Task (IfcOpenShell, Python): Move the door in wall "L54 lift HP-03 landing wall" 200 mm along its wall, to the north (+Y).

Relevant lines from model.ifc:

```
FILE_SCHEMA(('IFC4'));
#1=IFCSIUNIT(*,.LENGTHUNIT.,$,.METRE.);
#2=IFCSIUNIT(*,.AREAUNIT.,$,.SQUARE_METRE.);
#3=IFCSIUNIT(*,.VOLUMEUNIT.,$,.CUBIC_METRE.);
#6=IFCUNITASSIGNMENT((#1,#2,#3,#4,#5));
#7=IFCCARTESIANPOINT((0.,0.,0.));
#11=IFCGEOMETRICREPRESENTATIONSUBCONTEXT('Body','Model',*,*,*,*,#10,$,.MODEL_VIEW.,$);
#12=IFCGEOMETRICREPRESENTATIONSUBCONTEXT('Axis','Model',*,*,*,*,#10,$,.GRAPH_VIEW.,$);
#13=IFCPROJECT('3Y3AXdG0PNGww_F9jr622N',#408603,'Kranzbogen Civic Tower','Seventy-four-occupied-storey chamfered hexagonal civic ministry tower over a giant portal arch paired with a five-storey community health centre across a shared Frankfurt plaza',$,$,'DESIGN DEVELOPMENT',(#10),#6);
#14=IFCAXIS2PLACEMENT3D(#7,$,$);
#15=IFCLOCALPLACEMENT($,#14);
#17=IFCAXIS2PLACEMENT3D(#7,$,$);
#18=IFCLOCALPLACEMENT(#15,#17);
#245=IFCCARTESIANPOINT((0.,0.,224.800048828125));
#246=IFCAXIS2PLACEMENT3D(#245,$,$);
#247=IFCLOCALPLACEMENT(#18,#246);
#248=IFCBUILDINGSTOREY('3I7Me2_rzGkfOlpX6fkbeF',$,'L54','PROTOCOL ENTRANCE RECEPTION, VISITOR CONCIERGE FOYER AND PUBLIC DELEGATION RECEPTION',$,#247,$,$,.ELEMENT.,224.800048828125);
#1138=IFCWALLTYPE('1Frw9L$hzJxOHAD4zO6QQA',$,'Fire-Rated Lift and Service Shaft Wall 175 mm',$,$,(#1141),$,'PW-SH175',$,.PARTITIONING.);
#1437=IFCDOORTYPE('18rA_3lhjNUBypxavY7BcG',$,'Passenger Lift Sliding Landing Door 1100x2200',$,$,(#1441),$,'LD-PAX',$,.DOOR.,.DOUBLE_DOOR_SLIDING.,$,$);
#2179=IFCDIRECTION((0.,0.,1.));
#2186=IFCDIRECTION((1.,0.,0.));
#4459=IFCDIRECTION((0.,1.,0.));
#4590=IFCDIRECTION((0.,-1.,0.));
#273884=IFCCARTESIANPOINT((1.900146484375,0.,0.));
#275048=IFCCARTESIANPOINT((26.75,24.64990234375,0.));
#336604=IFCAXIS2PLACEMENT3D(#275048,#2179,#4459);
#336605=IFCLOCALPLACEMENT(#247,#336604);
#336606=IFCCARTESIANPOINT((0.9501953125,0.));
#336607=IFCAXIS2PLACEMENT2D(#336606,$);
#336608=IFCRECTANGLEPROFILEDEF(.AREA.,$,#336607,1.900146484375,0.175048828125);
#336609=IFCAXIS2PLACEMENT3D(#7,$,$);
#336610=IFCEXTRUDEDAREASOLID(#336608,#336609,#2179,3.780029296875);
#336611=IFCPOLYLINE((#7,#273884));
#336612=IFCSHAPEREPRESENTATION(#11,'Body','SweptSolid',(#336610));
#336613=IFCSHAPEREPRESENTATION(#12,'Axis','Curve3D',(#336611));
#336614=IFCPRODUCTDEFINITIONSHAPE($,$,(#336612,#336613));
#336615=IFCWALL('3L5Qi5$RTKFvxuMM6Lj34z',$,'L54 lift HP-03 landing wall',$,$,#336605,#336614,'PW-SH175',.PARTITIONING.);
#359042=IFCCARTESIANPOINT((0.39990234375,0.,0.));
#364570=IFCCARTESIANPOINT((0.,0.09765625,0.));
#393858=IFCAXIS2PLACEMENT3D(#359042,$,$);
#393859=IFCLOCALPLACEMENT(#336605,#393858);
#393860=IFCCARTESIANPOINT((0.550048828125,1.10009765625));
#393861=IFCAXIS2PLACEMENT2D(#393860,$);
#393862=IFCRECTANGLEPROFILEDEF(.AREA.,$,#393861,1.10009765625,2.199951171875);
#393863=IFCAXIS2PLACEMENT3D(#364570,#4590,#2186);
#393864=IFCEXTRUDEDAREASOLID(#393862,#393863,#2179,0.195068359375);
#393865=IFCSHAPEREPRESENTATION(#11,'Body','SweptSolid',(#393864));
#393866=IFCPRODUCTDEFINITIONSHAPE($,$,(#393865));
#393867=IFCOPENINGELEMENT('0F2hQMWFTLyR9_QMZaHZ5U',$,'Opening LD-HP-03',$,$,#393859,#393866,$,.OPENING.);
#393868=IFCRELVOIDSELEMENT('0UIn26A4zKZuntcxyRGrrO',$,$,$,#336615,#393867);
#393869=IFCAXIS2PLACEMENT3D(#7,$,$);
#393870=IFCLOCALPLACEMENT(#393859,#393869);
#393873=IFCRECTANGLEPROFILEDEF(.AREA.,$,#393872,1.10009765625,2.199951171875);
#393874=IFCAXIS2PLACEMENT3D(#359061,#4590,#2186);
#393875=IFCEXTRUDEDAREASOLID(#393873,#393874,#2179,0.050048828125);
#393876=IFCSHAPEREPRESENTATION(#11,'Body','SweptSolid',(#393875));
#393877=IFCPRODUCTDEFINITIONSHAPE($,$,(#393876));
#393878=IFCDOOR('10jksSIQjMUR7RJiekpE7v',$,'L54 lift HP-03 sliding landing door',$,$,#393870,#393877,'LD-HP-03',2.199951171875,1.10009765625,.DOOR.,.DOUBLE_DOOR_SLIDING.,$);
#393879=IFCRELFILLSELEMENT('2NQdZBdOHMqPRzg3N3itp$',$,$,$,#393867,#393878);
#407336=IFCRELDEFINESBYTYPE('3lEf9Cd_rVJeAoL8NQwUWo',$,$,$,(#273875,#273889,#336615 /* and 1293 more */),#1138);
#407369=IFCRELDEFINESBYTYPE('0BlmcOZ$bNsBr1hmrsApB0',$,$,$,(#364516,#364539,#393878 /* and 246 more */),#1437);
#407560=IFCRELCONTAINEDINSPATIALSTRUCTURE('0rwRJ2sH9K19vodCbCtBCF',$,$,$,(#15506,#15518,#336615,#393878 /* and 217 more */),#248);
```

```python
import ifcopenshell
import ifcopenshell.api.geometry
import ifcopenshell.util.placement

model = ifcopenshell.open("model.ifc")

door = model.by_guid("10jksSIQjMUR7RJiekpE7v")
opening = door.FillsVoids[0].RelatingOpeningElement
wall = opening.VoidsElements[0].RelatingBuildingElement

wall_matrix = ifcopenshell.util.placement.get_local_placement(wall.ObjectPlacement)
shift = wall_matrix[:3, 0] * 0.2
before = ifcopenshell.util.placement.get_local_placement(door.ObjectPlacement)[:3, 3].copy()

# The door is placed relative to its opening, so it follows when the opening moves.
matrix = ifcopenshell.util.placement.get_local_placement(opening.ObjectPlacement)
matrix[:3, 3] += shift
ifcopenshell.api.geometry.edit_object_placement(
    model, product=opening, matrix=matrix, is_si=False, should_transform_children=True
)

after = ifcopenshell.util.placement.get_local_placement(door.ObjectPlacement)[:3, 3]
print("door moved by", (after - before).round(3) + 0.0)

model.write("model_edited.ifc")
```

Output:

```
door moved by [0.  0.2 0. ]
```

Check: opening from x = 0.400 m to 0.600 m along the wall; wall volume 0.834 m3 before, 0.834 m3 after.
